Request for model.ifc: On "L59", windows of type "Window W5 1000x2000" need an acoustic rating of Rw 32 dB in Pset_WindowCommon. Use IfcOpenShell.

First a look at what the model holds.

```python
import ifcopenshell
import ifcopenshell.util.element

model = ifcopenshell.open("model.ifc")
print(model.schema)
storey = next(s for s in model.by_type("IfcBuildingStorey") if s.Name == "L59")
windows = [e for e in ifcopenshell.util.element.get_decomposition(storey) if e.is_a("IfcWindow")]
seen = {}
for e in windows:
    element_type = ifcopenshell.util.element.get_type(e)
    key = (element_type.Name if element_type != e and element_type else None, ifcopenshell.util.element.get_pset(e, "Pset_WindowCommon", "AcousticRating"))
    seen[key] = seen.get(key, 0) + 1
for (name, value), count in sorted(seen.items(), key=str):
    print(count, "x", name, "|", value)
```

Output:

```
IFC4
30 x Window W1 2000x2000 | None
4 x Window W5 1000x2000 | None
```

```python
import ifcopenshell
import ifcopenshell.api.pset
import ifcopenshell.util.element

model = ifcopenshell.open("model.ifc")

storey = next(s for s in model.by_type("IfcBuildingStorey") if s.Name == "L59")
windows = [e for e in ifcopenshell.util.element.get_decomposition(storey) if e.is_a("IfcWindow")]

count = 0
for e in windows:
    element_type = ifcopenshell.util.element.get_type(e)
    if element_type in (None, e) or element_type.Name != "Window W5 1000x2000":
        continue
    # add_pset returns the element's existing set when there is one.
    pset = ifcopenshell.api.pset.add_pset(model, product=e, name="Pset_WindowCommon")
    ifcopenshell.api.pset.edit_pset(model, pset=pset, properties={"AcousticRating": "Rw 32 dB"})
    count += 1

print(count, "windows updated")

model.write("model-out.ifc")
```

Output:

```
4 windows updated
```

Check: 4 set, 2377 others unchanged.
